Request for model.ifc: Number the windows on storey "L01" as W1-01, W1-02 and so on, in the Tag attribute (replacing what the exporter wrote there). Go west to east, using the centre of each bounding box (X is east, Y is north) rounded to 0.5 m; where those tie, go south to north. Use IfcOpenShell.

First a look at what the model holds.

```python
import ifcopenshell
import ifcopenshell.util.element
import ifcopenshell.util.placement

model = ifcopenshell.open("model.ifc")
print(model.schema)
storey = next(s for s in model.by_type("IfcBuildingStorey") if s.Name == "L01")
windows = [e for e in ifcopenshell.util.element.get_decomposition(storey) if e.is_a("IfcWindow")]
for e in sorted(windows, key=lambda e: e.id()):
    origin = ifcopenshell.util.placement.get_local_placement(e.ObjectPlacement)[:3, 3]
    print(e.id(), e.Tag, e.Name, origin.round(2) + 0.0, sep=" | ")
```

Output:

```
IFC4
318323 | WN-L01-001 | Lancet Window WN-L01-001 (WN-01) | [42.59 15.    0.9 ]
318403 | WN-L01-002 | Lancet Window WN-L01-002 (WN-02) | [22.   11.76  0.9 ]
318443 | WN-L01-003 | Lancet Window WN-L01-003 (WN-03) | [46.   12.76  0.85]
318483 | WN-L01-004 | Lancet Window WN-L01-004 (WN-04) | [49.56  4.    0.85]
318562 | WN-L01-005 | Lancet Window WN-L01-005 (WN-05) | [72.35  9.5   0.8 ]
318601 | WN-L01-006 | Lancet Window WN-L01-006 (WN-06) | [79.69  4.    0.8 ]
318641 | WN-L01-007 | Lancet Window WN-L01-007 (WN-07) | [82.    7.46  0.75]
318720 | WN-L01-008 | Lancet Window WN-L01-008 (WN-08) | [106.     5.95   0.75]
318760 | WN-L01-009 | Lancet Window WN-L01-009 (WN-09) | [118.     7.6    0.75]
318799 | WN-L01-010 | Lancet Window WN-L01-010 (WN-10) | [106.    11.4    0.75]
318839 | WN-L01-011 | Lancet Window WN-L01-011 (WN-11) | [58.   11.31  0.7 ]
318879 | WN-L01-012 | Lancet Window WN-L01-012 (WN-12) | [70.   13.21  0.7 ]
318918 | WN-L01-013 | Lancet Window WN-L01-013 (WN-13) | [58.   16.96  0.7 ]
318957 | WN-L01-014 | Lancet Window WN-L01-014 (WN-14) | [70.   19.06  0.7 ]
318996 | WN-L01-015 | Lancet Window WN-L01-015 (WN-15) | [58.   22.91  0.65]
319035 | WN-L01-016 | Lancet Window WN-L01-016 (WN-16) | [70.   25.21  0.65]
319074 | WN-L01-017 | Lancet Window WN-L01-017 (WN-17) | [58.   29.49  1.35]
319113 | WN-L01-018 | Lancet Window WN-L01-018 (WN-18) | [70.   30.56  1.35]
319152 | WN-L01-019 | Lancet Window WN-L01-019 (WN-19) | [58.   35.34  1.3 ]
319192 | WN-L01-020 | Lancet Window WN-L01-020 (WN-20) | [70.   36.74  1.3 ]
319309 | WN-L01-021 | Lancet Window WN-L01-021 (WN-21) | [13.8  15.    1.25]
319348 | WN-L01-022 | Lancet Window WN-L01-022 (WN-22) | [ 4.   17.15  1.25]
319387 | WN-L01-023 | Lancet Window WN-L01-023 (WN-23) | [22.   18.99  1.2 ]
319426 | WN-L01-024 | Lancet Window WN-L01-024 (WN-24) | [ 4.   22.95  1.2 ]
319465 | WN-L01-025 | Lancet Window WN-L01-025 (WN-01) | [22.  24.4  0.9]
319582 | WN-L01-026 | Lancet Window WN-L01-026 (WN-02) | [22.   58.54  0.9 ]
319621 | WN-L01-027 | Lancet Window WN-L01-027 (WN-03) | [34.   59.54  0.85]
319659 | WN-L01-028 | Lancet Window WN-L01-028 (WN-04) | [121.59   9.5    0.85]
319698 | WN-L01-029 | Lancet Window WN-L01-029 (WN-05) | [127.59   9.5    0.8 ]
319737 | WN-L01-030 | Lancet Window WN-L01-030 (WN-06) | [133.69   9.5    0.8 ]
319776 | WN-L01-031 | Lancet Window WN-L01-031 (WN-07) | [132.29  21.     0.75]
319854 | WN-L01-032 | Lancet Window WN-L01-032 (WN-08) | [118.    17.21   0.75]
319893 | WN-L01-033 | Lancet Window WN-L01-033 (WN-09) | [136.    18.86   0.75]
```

```python
import ifcopenshell
import ifcopenshell.geom
import ifcopenshell.util.element
import ifcopenshell.util.shape

model = ifcopenshell.open("model.ifc")
settings = ifcopenshell.geom.settings()
settings.set("use-world-coords", True)


def centre(element):
    shape = ifcopenshell.geom.create_shape(settings, element)
    return ifcopenshell.util.shape.get_bbox_centroid(shape.geometry)


storey = next(s for s in model.by_type("IfcBuildingStorey") if s.Name == "L01")
windows = [e for e in ifcopenshell.util.element.get_decomposition(storey) if e.is_a("IfcWindow")]

# Insertion points can sit at a corner or the storey origin, so sort by the geometry (in metres).
centres = {e: centre(e) for e in windows}
windows.sort(key=lambda e: (round(centres[e][0] / 0.5), centres[e][1]))

for i, e in enumerate(windows, start=1):
    number = f"W1-{i:02d}"
    e.Tag = number
    print(e.id(), number)

model.write("model_rev.ifc")
```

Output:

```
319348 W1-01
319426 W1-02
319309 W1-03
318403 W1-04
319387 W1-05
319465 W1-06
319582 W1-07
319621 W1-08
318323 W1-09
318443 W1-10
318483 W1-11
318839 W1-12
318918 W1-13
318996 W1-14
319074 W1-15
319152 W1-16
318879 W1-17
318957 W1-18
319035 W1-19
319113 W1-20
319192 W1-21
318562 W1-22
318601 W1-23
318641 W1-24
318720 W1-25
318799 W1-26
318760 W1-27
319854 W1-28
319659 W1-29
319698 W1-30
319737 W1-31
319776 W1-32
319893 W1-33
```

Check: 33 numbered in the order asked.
